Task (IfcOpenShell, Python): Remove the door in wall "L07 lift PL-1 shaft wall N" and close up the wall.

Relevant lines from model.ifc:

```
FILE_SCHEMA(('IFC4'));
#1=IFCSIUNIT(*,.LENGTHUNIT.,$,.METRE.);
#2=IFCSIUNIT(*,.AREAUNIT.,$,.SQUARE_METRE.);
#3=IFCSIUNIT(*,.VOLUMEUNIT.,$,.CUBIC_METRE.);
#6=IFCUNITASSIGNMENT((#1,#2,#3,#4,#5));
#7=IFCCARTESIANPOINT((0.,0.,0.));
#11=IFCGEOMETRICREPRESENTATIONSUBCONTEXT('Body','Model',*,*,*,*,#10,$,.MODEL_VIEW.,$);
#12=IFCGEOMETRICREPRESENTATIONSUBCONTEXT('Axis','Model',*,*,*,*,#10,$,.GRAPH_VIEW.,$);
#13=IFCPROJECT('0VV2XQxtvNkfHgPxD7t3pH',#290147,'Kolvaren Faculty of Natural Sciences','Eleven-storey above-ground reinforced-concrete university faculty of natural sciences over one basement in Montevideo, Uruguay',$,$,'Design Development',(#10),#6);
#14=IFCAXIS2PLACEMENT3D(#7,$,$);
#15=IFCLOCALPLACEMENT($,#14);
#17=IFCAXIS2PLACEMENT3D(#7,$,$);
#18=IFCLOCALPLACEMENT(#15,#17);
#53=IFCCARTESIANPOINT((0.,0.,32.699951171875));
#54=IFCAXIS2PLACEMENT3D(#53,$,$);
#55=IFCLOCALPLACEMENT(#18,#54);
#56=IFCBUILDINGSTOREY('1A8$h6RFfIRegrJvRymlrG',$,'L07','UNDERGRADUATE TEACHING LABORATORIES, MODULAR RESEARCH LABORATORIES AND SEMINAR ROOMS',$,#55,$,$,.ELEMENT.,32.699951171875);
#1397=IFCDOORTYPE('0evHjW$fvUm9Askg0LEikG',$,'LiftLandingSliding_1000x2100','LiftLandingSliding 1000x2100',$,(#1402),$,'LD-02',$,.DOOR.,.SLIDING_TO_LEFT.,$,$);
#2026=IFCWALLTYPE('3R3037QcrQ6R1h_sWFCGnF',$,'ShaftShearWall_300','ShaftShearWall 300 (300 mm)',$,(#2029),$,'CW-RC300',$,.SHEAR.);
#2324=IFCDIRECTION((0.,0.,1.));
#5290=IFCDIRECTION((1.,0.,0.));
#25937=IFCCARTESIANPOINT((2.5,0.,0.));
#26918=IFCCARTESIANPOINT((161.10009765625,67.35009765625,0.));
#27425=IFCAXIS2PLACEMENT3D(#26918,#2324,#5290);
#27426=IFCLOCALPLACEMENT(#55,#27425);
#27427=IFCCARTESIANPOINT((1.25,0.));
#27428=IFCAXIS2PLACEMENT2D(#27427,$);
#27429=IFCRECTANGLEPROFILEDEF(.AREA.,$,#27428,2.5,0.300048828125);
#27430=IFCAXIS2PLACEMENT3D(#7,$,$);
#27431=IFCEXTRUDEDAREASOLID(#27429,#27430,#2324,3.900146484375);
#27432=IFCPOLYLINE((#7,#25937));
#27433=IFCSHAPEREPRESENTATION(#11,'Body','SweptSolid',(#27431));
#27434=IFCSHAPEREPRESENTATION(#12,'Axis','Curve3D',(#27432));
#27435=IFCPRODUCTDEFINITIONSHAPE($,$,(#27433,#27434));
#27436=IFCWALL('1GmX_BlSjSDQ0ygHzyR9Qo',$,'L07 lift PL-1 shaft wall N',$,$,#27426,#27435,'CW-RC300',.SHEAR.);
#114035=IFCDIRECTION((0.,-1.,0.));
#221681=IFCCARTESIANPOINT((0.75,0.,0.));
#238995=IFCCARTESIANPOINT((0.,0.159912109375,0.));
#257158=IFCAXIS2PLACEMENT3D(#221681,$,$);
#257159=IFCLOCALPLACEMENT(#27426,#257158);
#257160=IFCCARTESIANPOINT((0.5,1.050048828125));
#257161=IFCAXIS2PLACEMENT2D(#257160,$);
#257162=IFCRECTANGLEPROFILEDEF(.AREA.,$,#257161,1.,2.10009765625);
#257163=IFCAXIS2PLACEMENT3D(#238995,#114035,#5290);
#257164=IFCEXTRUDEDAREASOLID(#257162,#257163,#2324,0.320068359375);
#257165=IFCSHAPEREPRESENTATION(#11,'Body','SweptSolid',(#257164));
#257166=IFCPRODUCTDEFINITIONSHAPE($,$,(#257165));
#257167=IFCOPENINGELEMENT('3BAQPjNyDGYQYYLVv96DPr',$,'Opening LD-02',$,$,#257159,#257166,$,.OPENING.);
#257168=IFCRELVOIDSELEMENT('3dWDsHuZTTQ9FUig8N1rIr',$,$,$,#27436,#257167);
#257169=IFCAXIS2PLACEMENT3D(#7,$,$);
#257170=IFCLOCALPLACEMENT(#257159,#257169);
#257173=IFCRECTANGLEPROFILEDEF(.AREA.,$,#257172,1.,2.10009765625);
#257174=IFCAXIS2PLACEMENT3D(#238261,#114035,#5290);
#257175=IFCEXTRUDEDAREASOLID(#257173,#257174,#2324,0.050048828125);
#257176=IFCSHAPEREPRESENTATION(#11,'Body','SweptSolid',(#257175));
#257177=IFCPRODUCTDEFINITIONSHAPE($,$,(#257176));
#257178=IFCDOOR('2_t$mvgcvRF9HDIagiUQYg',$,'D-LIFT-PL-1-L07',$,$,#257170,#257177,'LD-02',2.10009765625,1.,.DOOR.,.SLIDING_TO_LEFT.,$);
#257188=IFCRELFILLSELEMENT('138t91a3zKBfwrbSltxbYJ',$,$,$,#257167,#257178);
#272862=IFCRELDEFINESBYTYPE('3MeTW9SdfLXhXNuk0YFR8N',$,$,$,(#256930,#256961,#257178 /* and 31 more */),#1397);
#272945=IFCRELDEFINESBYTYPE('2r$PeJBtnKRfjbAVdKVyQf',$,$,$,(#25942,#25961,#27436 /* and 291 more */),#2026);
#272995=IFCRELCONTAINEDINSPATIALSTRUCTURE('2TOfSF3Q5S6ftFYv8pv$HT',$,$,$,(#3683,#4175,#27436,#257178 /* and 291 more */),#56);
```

```python
import ifcopenshell
import ifcopenshell.api.feature
import ifcopenshell.api.root
import ifcopenshell.geom
import ifcopenshell.util.shape

model = ifcopenshell.open("model.ifc")
settings = ifcopenshell.geom.settings()


def volume(element):
    """Net volume in cubic metres, openings subtracted."""
    shape = ifcopenshell.geom.create_shape(settings, element)
    return ifcopenshell.util.shape.get_volume(shape.geometry)


door = model.by_id(257178)
opening = door.FillsVoids[0].RelatingOpeningElement
wall = opening.VoidsElements[0].RelatingBuildingElement
before = volume(wall)

ifcopenshell.api.root.remove_product(model, product=door)
ifcopenshell.api.feature.remove_feature(model, feature=opening)

after = volume(wall)

print(f"wall volume {before:.3f} -> {after:.3f} m3")

model.write("model_edited.ifc")
```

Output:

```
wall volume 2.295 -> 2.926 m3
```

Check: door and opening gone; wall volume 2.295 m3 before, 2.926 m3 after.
